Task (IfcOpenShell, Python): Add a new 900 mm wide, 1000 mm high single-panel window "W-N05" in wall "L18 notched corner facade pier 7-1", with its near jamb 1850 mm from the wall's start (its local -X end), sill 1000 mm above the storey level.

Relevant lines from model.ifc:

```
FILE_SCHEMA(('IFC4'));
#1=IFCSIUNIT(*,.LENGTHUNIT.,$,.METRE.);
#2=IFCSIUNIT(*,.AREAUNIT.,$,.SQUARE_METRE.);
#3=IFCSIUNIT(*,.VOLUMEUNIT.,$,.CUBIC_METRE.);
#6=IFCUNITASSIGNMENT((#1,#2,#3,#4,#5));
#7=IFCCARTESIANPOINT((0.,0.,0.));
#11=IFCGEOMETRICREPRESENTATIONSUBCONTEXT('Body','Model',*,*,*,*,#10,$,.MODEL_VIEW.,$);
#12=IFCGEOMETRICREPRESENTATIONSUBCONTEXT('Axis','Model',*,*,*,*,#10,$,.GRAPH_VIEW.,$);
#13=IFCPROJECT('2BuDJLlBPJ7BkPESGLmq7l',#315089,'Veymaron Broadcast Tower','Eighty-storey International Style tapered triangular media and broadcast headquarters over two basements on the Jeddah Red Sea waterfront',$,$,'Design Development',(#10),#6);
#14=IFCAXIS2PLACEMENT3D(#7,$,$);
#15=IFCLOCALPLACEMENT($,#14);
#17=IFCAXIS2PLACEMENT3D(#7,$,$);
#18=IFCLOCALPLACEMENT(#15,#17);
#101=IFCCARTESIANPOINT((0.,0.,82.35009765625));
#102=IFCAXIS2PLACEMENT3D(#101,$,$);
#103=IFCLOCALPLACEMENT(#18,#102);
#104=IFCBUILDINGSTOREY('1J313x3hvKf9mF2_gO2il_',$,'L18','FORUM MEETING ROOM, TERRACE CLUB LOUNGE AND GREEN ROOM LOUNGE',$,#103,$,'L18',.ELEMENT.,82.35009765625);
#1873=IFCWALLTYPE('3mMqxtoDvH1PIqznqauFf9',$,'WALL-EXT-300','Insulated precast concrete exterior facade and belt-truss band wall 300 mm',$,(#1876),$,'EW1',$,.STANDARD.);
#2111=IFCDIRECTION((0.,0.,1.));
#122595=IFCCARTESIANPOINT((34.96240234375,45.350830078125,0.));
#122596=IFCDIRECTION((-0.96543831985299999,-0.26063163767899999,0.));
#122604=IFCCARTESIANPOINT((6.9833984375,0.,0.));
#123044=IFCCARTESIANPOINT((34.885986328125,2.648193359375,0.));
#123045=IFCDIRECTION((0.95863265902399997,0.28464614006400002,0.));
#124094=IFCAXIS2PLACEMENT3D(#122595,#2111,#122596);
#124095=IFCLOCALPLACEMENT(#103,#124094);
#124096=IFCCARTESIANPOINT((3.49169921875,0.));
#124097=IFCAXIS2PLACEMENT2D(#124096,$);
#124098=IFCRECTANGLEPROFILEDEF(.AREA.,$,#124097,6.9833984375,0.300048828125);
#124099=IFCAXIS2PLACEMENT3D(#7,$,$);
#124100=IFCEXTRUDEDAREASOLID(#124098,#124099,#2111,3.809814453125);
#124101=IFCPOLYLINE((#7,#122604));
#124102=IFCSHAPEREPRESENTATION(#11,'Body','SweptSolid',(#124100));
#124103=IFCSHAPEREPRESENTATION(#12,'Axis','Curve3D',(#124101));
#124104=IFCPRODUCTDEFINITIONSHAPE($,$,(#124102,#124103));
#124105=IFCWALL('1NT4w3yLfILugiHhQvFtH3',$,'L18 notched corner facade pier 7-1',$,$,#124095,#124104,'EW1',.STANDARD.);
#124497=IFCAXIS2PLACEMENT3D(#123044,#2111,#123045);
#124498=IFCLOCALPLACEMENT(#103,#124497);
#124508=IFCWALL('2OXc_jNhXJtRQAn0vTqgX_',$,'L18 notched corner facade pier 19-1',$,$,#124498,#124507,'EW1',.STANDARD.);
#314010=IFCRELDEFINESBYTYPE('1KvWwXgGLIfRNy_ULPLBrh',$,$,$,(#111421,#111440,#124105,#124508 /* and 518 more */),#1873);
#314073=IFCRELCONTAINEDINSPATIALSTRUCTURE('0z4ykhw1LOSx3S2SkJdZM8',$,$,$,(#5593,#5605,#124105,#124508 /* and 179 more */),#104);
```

```python
import numpy as np
import ifcopenshell
import ifcopenshell.api.feature
import ifcopenshell.api.geometry
import ifcopenshell.api.root
import ifcopenshell.api.spatial
import ifcopenshell.geom
import ifcopenshell.util.element
import ifcopenshell.util.placement
import ifcopenshell.util.representation
import ifcopenshell.util.shape
import ifcopenshell.util.unit

model = ifcopenshell.open("model.ifc")
unit_scale = ifcopenshell.util.unit.calculate_unit_scale(model)
settings = ifcopenshell.geom.settings()


def volume(element):
    """Net volume in cubic metres, openings subtracted."""
    shape = ifcopenshell.geom.create_shape(settings, element)
    return ifcopenshell.util.shape.get_volume(shape.geometry)


wall = model.by_guid("1NT4w3yLfILugiHhQvFtH3")
storey = ifcopenshell.util.element.get_container(wall, ifc_class="IfcBuildingStorey")
context = ifcopenshell.util.representation.get_context(model, "Model", "Body", "MODEL_VIEW")
before = volume(wall)

width, height, from_end, sill = 0.9, 1, 1.85, 1  # metres

# The wall runs along its own X axis, and the end named is its -X end.
wall_shape = ifcopenshell.geom.create_shape(settings, wall)
x, y, z = ifcopenshell.util.shape.get_vertices(wall_shape.geometry).T
start = x.min() + from_end
face, thickness = float(y.min()), float(y.max() - y.min())
wall_matrix = ifcopenshell.util.placement.get_local_placement(wall.ObjectPlacement)
level = ifcopenshell.util.placement.get_local_placement(storey.ObjectPlacement)[2, 3]


def in_wall(x, y):
    """Placement at x, y metres in the wall's axes, at sill height."""
    matrix = wall_matrix.copy()
    matrix[:, 3] = wall_matrix @ np.array([x / unit_scale, y / unit_scale, 0.0, 1.0])
    matrix[2, 3] = level + sill / unit_scale
    return matrix


# Opening: a box that overshoots both wall faces by 50 mm.
opening = ifcopenshell.api.root.create_entity(model, ifc_class="IfcOpeningElement", predefined_type="OPENING")
box = ifcopenshell.api.geometry.add_wall_representation(
    model, context=context, length=width, height=height, thickness=thickness + 0.1
)
ifcopenshell.api.geometry.assign_representation(model, product=opening, representation=box)
ifcopenshell.api.geometry.edit_object_placement(model, product=opening, matrix=in_wall(start, face - 0.05), is_si=False)
ifcopenshell.api.feature.add_feature(model, feature=opening, element=wall)

window = ifcopenshell.api.root.create_entity(model, ifc_class="IfcWindow", name="W-N05", predefined_type="WINDOW")
window.OverallWidth, window.OverallHeight = width / unit_scale, height / unit_scale
window.PartitioningType = "SINGLE_PANEL"
body = ifcopenshell.api.geometry.add_window_representation(
    model,
    context=context,
    overall_width=window.OverallWidth,
    overall_height=window.OverallHeight,
    partition_type="SINGLE_PANEL",
)
ifcopenshell.api.geometry.assign_representation(model, product=window, representation=body)
ifcopenshell.api.spatial.assign_container(model, products=[window], relating_structure=storey)
ifcopenshell.api.feature.add_filling(model, opening=opening, element=window)

# Centre the window in the wall's thickness.
ifcopenshell.api.geometry.edit_object_placement(model, product=window, matrix=in_wall(start, face), is_si=False)
window_shape = ifcopenshell.geom.create_shape(settings, window)
depth = ifcopenshell.util.shape.get_vertices(window_shape.geometry)[:, 1]
offset = face + thickness / 2 - (depth.min() + depth.max()) / 2
ifcopenshell.api.geometry.edit_object_placement(model, product=window, matrix=in_wall(start, offset), is_si=False)

after = volume(wall)

print(f"wall volume {before:.3f} -> {after:.3f} m3")

model.write("model-out.ifc")
```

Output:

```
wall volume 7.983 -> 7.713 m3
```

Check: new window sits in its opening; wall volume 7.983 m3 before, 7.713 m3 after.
